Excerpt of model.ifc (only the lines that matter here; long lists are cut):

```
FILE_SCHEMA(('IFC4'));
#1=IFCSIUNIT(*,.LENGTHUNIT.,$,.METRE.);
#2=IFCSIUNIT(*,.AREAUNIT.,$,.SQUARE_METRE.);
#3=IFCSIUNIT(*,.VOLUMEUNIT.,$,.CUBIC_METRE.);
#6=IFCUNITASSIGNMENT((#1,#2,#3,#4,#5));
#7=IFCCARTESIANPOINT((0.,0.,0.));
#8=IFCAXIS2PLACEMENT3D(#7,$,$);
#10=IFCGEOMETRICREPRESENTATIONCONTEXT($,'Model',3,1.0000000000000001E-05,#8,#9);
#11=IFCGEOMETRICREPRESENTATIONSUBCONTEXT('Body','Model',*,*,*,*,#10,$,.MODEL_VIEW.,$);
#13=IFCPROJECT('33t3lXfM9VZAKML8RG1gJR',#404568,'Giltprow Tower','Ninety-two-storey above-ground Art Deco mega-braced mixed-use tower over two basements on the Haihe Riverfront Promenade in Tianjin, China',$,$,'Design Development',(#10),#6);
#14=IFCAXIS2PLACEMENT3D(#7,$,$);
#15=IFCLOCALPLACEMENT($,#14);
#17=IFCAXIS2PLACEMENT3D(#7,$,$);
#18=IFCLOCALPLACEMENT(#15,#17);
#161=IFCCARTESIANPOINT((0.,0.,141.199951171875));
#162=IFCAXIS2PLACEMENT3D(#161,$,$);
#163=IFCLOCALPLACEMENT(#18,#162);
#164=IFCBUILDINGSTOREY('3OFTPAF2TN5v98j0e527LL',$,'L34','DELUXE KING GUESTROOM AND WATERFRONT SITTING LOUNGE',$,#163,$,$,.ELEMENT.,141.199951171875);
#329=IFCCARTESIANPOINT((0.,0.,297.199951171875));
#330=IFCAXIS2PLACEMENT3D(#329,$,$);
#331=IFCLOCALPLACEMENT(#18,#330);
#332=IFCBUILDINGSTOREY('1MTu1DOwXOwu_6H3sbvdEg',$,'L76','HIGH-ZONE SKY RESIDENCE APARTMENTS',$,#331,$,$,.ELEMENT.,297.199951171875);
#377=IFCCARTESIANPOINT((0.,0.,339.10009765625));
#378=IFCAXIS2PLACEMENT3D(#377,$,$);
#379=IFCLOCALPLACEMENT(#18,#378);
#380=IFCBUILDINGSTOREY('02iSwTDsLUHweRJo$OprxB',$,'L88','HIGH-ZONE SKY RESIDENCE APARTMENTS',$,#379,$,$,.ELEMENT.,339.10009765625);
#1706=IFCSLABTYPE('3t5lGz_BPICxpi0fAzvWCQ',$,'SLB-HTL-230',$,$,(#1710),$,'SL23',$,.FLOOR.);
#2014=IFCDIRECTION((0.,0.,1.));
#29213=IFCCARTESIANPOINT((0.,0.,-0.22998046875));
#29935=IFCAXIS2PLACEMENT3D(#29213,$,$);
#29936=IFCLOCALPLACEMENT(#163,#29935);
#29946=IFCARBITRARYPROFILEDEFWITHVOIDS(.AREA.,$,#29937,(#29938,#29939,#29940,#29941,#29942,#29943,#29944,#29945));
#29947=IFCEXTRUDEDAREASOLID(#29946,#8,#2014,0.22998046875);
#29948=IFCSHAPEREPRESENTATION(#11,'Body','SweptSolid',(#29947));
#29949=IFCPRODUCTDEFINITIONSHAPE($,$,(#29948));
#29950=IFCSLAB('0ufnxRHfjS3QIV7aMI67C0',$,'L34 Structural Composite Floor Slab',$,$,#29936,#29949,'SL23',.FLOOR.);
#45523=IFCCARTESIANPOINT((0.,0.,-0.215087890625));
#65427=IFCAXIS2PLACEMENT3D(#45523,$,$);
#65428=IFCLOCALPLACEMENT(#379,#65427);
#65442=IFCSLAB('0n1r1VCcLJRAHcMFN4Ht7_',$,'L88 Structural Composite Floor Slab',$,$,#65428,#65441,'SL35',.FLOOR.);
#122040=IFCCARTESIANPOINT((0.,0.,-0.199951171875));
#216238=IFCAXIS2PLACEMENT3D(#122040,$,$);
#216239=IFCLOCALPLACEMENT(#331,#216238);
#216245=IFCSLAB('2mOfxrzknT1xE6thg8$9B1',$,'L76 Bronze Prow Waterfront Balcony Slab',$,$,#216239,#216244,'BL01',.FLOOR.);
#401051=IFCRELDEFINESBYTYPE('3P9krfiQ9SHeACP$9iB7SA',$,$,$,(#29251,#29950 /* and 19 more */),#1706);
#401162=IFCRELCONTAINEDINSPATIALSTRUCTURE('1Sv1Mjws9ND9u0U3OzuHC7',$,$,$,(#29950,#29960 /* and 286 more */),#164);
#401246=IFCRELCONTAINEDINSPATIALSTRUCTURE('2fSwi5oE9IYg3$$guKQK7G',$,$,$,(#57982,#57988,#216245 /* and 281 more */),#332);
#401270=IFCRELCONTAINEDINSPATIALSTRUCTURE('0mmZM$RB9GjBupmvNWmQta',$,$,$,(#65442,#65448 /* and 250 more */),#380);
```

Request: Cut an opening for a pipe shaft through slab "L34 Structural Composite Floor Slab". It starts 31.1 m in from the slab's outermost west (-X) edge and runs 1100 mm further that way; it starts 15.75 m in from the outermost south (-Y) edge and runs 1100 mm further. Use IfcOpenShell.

```python
import numpy as np
import ifcopenshell
import ifcopenshell.api.feature
import ifcopenshell.api.geometry
import ifcopenshell.api.root
import ifcopenshell.geom
import ifcopenshell.util.placement
import ifcopenshell.util.representation
import ifcopenshell.util.shape
import ifcopenshell.util.unit

model = ifcopenshell.open("model.ifc")
unit_scale = ifcopenshell.util.unit.calculate_unit_scale(model)
settings = ifcopenshell.geom.settings()


def volume(element):
    """Net volume in cubic metres, openings subtracted."""
    shape = ifcopenshell.geom.create_shape(settings, element)
    return ifcopenshell.util.shape.get_volume(shape.geometry)


slab = model.by_id(29950)
before = volume(slab)

# Extent in the slab's own axes, in metres. The edges named are its -X and -Y sides.
slab_shape = ifcopenshell.geom.create_shape(settings, slab)
vertices = ifcopenshell.util.shape.get_vertices(slab_shape.geometry)
x_min, y_min, bottom = vertices.min(axis=0)
top = vertices[:, 2].max()

opening = ifcopenshell.api.root.create_entity(model, ifc_class="IfcOpeningElement", name="Pipe shaft opening", predefined_type="OPENING")
context = ifcopenshell.util.representation.get_context(model, "Model", "Body", "MODEL_VIEW")
width, depth = 1.1, 1.1
outline = [(0.0, 0.0), (width, 0.0), (width, depth), (0.0, depth), (0.0, 0.0)]
# Overshoot both faces by 50 mm so the cut is clean.
shape = ifcopenshell.api.geometry.add_slab_representation(
    model, context=context, depth=top - bottom + 0.1, polyline=outline
)
ifcopenshell.api.geometry.assign_representation(model, product=opening, representation=shape)

matrix = ifcopenshell.util.placement.get_local_placement(slab.ObjectPlacement)
matrix[:, 3] = matrix @ np.append(np.array([x_min + 31.1, y_min + 15.75, bottom - 0.05]) / unit_scale, 1.0)
ifcopenshell.api.geometry.edit_object_placement(model, product=opening, matrix=matrix, is_si=False)
ifcopenshell.api.feature.add_feature(model, feature=opening, element=slab)

after = volume(slab)

print(f"slab volume {before:.3f} -> {after:.3f} m3")

model.write("model-out.ifc")
```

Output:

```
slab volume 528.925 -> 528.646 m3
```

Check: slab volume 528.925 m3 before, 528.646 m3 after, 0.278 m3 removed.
